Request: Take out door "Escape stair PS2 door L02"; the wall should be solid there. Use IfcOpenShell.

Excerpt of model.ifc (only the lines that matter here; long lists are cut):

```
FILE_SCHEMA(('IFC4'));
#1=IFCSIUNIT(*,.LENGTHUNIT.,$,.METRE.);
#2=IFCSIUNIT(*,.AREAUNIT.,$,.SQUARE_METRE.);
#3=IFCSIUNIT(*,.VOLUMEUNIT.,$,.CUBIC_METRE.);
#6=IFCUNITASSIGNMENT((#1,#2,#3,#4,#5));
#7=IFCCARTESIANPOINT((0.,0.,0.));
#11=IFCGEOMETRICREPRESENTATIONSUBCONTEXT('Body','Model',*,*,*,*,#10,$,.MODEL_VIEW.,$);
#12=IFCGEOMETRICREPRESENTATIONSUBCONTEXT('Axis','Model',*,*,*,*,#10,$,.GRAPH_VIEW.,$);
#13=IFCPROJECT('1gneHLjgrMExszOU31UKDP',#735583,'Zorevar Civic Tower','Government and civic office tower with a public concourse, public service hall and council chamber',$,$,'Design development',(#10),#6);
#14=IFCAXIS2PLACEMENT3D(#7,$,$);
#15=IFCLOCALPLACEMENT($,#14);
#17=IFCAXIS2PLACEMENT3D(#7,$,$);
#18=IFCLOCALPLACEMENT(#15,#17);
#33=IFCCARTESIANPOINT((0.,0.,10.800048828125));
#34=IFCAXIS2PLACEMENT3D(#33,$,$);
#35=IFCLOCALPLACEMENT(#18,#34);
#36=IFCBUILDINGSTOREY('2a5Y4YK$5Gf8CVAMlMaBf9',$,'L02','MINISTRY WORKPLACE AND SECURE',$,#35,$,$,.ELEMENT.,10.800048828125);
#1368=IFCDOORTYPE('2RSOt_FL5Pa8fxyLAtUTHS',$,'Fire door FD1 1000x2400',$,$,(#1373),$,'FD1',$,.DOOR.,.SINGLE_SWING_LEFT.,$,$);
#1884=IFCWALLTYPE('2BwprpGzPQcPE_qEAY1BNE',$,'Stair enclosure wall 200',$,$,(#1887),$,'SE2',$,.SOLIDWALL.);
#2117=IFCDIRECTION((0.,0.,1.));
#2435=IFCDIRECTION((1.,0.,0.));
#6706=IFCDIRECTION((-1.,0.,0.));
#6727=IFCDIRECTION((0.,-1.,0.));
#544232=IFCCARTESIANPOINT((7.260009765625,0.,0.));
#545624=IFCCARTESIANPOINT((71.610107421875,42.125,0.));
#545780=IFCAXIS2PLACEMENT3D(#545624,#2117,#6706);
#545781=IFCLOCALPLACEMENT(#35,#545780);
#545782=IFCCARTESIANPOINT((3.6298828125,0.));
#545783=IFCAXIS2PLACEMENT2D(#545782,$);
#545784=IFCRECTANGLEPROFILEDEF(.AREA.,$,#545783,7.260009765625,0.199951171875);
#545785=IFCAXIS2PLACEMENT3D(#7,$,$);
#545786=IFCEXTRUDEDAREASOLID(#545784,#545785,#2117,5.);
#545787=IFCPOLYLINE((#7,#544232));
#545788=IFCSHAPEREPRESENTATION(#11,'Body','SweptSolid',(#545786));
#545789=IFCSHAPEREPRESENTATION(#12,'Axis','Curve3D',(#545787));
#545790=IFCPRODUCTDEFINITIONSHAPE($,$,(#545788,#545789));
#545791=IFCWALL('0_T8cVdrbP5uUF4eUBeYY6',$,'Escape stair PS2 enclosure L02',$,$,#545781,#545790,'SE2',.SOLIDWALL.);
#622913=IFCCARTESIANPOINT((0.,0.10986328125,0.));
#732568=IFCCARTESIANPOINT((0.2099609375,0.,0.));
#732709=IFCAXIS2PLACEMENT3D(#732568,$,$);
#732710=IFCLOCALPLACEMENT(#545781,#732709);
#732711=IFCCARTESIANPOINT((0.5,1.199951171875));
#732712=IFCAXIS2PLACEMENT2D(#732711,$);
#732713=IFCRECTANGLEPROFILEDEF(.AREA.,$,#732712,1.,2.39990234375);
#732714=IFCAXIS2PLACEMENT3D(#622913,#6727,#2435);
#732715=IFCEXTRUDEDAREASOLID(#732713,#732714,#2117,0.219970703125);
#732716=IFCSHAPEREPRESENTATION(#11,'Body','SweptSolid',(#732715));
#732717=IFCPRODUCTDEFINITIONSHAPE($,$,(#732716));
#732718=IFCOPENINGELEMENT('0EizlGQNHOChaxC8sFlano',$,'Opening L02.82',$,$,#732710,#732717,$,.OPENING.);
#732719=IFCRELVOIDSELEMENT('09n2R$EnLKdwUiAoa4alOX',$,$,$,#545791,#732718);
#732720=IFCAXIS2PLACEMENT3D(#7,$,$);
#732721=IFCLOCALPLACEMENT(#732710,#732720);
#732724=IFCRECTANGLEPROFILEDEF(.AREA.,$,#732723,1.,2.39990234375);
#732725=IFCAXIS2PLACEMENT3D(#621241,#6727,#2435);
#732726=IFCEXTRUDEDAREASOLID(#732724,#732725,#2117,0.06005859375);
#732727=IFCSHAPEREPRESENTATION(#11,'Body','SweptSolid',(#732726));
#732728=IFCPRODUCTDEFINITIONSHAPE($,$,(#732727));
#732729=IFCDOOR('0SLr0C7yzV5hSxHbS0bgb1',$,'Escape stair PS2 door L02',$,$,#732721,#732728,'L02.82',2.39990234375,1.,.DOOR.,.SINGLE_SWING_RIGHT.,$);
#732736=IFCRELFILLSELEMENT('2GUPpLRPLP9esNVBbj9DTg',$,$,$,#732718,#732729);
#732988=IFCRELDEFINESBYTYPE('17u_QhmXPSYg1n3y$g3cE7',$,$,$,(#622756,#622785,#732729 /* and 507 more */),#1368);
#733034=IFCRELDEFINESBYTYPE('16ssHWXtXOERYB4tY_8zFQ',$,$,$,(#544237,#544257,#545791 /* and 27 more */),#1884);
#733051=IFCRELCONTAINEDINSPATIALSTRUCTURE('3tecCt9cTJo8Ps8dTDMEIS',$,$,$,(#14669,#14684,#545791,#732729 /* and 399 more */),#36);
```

```python
import ifcopenshell
import ifcopenshell.api.feature
import ifcopenshell.api.root
import ifcopenshell.geom
import ifcopenshell.util.shape

model = ifcopenshell.open("model.ifc")
settings = ifcopenshell.geom.settings()


def volume(element):
    """Net volume in cubic metres, openings subtracted."""
    shape = ifcopenshell.geom.create_shape(settings, element)
    return ifcopenshell.util.shape.get_volume(shape.geometry)


door = model.by_guid("0SLr0C7yzV5hSxHbS0bgb1")
opening = door.FillsVoids[0].RelatingOpeningElement
wall = opening.VoidsElements[0].RelatingBuildingElement
before = volume(wall)

ifcopenshell.api.root.remove_product(model, product=door)
ifcopenshell.api.feature.remove_feature(model, feature=opening)

after = volume(wall)

print(f"wall volume {before:.3f} -> {after:.3f} m3")

model.write("model-out.ifc")
```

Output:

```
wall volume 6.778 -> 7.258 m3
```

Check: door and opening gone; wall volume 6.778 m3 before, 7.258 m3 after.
